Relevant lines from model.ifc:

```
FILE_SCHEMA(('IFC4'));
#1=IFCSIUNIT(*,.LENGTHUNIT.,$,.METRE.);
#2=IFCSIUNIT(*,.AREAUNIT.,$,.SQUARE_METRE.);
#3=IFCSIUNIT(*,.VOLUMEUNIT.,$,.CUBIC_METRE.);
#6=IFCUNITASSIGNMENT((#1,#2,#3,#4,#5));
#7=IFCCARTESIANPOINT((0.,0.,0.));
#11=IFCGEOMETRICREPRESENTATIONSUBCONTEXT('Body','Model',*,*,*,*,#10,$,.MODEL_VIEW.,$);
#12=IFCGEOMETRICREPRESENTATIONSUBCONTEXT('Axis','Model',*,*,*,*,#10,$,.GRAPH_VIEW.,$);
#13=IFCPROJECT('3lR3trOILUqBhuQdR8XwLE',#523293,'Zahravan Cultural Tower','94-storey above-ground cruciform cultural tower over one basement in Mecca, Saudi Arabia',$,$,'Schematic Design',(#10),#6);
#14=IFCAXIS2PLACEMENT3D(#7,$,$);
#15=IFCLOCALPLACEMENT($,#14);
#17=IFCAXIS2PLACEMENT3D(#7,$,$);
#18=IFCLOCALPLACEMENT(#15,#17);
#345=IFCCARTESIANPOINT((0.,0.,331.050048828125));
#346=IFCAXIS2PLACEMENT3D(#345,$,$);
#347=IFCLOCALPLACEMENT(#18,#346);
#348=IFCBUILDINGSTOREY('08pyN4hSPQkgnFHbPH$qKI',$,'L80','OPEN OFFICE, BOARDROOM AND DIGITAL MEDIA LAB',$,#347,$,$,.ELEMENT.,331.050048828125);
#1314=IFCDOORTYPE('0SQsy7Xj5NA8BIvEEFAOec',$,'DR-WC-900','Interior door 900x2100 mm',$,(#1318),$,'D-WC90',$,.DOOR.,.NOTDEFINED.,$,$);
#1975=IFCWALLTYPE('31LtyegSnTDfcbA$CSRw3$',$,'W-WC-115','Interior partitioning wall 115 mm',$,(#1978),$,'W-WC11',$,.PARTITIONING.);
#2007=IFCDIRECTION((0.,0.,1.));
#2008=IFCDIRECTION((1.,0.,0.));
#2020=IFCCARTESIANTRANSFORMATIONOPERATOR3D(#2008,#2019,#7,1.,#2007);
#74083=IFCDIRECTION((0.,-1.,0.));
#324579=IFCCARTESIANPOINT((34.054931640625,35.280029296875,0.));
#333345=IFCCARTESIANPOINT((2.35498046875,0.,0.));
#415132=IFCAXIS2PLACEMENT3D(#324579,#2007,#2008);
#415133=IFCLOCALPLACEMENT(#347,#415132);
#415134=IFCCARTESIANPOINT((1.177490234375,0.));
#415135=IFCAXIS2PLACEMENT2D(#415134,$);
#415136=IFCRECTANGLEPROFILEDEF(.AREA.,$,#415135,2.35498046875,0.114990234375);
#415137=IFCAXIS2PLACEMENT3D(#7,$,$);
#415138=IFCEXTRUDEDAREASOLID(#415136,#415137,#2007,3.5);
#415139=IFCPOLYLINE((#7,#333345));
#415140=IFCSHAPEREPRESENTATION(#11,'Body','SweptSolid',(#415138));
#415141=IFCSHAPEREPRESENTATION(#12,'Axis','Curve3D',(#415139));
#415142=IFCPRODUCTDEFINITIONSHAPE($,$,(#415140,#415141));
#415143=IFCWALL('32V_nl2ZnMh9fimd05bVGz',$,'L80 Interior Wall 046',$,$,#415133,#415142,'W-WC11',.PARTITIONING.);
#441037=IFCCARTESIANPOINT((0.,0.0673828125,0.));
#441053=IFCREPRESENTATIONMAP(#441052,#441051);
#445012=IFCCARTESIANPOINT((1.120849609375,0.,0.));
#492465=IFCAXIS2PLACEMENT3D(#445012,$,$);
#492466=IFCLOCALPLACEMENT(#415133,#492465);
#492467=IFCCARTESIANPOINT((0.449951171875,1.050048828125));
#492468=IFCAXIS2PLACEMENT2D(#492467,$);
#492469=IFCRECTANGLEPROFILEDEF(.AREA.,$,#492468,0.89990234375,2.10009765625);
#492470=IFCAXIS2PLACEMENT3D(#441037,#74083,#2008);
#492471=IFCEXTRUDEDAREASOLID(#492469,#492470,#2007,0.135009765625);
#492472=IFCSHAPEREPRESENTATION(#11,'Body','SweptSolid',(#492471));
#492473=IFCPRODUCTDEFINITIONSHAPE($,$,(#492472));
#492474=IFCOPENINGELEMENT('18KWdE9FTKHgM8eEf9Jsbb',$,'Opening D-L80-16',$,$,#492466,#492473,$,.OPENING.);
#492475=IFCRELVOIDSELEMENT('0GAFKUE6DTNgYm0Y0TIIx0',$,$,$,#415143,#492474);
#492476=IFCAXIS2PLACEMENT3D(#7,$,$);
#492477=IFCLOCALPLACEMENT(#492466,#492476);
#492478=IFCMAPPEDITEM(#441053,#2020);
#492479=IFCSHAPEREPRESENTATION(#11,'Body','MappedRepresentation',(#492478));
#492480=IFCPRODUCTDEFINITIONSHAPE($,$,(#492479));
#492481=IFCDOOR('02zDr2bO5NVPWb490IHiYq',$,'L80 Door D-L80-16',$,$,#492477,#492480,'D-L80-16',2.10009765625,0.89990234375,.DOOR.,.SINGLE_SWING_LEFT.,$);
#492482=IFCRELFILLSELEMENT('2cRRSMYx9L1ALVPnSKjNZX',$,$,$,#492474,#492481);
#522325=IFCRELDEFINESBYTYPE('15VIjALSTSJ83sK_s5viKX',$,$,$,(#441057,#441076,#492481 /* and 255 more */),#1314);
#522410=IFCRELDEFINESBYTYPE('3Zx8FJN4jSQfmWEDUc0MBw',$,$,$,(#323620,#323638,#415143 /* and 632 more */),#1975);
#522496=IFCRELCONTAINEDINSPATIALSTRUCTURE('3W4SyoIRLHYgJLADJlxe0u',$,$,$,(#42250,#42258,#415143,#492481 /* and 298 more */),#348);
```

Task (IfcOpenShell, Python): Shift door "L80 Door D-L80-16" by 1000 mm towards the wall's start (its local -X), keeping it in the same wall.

```python
import ifcopenshell
import ifcopenshell.api.geometry
import ifcopenshell.util.placement
import ifcopenshell.util.unit

model = ifcopenshell.open("model.ifc")
unit_scale = ifcopenshell.util.unit.calculate_unit_scale(model)

door = model.by_guid("02zDr2bO5NVPWb490IHiYq")
opening = door.FillsVoids[0].RelatingOpeningElement
wall = opening.VoidsElements[0].RelatingBuildingElement

wall_matrix = ifcopenshell.util.placement.get_local_placement(wall.ObjectPlacement)
shift = wall_matrix[:3, 0] * -1 / unit_scale
before = ifcopenshell.util.placement.get_local_placement(door.ObjectPlacement)[:3, 3].copy()

# The door is placed relative to its opening, so it follows when the opening moves.
matrix = ifcopenshell.util.placement.get_local_placement(opening.ObjectPlacement)
matrix[:3, 3] += shift
ifcopenshell.api.geometry.edit_object_placement(
    model, product=opening, matrix=matrix, is_si=False, should_transform_children=True
)

after = ifcopenshell.util.placement.get_local_placement(door.ObjectPlacement)[:3, 3]
print("door moved by", (after - before).round(3) + 0.0)

model.write("model_v2.ifc")
```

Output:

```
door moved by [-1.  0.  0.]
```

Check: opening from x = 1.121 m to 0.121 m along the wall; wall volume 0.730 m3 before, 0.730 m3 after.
